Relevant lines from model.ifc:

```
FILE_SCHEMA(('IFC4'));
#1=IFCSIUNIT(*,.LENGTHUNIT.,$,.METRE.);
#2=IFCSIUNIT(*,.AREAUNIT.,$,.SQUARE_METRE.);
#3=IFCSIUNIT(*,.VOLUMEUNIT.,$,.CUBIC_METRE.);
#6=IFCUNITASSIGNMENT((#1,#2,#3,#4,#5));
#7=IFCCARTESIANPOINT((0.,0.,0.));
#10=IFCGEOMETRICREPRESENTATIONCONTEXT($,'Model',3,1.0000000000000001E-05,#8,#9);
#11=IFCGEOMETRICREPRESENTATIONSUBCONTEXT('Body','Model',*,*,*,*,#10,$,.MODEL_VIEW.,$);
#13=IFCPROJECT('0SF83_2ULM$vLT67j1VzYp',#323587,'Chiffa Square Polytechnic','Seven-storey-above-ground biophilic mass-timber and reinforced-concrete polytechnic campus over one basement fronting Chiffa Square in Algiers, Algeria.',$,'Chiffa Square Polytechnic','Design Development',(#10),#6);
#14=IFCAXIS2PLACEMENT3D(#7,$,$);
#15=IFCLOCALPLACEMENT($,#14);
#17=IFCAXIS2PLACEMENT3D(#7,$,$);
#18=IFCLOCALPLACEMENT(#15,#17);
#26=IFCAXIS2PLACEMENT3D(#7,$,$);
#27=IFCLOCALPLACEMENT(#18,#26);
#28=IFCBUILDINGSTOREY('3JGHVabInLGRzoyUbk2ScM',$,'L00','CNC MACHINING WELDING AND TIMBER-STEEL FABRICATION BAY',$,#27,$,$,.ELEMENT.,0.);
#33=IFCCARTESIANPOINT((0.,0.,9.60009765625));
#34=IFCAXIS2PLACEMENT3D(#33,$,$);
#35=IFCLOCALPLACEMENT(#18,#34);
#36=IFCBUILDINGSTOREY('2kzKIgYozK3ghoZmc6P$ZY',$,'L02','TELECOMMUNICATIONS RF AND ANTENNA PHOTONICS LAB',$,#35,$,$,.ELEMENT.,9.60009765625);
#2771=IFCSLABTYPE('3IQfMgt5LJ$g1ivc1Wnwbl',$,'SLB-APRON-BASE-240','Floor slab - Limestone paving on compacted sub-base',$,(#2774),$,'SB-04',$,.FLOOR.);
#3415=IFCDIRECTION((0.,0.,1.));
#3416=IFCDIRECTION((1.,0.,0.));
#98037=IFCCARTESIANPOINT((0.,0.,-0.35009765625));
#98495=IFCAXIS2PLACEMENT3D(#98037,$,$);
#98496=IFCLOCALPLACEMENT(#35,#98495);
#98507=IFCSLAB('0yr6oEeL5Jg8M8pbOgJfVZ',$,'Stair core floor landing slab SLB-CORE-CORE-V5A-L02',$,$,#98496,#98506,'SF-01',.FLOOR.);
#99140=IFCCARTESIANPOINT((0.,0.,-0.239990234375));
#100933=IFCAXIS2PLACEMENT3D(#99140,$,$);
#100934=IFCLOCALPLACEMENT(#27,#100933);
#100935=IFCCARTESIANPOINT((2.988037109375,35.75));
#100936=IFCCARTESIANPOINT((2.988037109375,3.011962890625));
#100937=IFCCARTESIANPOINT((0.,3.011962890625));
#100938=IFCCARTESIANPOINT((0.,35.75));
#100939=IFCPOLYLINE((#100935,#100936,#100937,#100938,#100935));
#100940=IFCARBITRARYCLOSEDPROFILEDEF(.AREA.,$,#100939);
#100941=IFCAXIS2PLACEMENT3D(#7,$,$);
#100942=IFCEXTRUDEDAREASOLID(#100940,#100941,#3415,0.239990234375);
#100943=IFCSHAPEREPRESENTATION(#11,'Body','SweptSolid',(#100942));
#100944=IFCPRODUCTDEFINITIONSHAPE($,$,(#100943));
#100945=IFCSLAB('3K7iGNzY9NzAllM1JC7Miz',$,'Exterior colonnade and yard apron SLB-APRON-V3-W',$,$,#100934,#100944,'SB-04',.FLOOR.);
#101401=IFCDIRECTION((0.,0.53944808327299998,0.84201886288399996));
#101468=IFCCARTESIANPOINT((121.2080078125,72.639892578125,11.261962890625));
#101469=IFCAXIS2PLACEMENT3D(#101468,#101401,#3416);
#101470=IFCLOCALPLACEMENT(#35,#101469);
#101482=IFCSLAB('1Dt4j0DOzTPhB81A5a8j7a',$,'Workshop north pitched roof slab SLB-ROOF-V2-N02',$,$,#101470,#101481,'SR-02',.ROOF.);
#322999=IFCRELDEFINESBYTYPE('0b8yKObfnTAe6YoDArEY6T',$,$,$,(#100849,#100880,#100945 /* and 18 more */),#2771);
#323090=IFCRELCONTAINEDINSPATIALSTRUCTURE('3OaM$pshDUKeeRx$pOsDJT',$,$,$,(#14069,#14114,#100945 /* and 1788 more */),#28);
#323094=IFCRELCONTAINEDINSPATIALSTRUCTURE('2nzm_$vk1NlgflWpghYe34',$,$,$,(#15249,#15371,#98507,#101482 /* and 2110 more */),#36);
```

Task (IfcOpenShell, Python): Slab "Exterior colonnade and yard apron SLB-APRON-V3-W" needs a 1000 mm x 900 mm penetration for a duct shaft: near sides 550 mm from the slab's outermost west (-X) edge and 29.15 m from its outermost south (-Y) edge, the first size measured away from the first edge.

```python
import numpy as np
import ifcopenshell
import ifcopenshell.api.feature
import ifcopenshell.api.geometry
import ifcopenshell.api.root
import ifcopenshell.geom
import ifcopenshell.util.placement
import ifcopenshell.util.representation
import ifcopenshell.util.shape
import ifcopenshell.util.unit

model = ifcopenshell.open("model.ifc")
unit_scale = ifcopenshell.util.unit.calculate_unit_scale(model)
settings = ifcopenshell.geom.settings()


def volume(element):
    """Net volume in cubic metres, openings subtracted."""
    shape = ifcopenshell.geom.create_shape(settings, element)
    return ifcopenshell.util.shape.get_volume(shape.geometry)


slab = model.by_guid("3K7iGNzY9NzAllM1JC7Miz")
before = volume(slab)

# Extent in the slab's own axes, in metres. The edges named are its -X and -Y sides.
slab_shape = ifcopenshell.geom.create_shape(settings, slab)
vertices = ifcopenshell.util.shape.get_vertices(slab_shape.geometry)
x_min, y_min, bottom = vertices.min(axis=0)
top = vertices[:, 2].max()

opening = ifcopenshell.api.root.create_entity(model, ifc_class="IfcOpeningElement", name="Duct shaft opening", predefined_type="OPENING")
context = ifcopenshell.util.representation.get_context(model, "Model", "Body", "MODEL_VIEW")
width, depth = 1, 0.9
outline = [(0.0, 0.0), (width, 0.0), (width, depth), (0.0, depth), (0.0, 0.0)]
# Overshoot both faces by 50 mm so the cut is clean.
shape = ifcopenshell.api.geometry.add_slab_representation(
    model, context=context, depth=top - bottom + 0.1, polyline=outline
)
ifcopenshell.api.geometry.assign_representation(model, product=opening, representation=shape)

matrix = ifcopenshell.util.placement.get_local_placement(slab.ObjectPlacement)
matrix[:, 3] = matrix @ np.append(np.array([x_min + 0.55, y_min + 29.15, bottom - 0.05]) / unit_scale, 1.0)
ifcopenshell.api.geometry.edit_object_placement(model, product=opening, matrix=matrix, is_si=False)
ifcopenshell.api.feature.add_feature(model, feature=opening, element=slab)

after = volume(slab)

print(f"slab volume {before:.3f} -> {after:.3f} m3")

model.write("model_rev.ifc")
```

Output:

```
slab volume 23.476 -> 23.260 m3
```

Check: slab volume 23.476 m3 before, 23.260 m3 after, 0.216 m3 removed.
